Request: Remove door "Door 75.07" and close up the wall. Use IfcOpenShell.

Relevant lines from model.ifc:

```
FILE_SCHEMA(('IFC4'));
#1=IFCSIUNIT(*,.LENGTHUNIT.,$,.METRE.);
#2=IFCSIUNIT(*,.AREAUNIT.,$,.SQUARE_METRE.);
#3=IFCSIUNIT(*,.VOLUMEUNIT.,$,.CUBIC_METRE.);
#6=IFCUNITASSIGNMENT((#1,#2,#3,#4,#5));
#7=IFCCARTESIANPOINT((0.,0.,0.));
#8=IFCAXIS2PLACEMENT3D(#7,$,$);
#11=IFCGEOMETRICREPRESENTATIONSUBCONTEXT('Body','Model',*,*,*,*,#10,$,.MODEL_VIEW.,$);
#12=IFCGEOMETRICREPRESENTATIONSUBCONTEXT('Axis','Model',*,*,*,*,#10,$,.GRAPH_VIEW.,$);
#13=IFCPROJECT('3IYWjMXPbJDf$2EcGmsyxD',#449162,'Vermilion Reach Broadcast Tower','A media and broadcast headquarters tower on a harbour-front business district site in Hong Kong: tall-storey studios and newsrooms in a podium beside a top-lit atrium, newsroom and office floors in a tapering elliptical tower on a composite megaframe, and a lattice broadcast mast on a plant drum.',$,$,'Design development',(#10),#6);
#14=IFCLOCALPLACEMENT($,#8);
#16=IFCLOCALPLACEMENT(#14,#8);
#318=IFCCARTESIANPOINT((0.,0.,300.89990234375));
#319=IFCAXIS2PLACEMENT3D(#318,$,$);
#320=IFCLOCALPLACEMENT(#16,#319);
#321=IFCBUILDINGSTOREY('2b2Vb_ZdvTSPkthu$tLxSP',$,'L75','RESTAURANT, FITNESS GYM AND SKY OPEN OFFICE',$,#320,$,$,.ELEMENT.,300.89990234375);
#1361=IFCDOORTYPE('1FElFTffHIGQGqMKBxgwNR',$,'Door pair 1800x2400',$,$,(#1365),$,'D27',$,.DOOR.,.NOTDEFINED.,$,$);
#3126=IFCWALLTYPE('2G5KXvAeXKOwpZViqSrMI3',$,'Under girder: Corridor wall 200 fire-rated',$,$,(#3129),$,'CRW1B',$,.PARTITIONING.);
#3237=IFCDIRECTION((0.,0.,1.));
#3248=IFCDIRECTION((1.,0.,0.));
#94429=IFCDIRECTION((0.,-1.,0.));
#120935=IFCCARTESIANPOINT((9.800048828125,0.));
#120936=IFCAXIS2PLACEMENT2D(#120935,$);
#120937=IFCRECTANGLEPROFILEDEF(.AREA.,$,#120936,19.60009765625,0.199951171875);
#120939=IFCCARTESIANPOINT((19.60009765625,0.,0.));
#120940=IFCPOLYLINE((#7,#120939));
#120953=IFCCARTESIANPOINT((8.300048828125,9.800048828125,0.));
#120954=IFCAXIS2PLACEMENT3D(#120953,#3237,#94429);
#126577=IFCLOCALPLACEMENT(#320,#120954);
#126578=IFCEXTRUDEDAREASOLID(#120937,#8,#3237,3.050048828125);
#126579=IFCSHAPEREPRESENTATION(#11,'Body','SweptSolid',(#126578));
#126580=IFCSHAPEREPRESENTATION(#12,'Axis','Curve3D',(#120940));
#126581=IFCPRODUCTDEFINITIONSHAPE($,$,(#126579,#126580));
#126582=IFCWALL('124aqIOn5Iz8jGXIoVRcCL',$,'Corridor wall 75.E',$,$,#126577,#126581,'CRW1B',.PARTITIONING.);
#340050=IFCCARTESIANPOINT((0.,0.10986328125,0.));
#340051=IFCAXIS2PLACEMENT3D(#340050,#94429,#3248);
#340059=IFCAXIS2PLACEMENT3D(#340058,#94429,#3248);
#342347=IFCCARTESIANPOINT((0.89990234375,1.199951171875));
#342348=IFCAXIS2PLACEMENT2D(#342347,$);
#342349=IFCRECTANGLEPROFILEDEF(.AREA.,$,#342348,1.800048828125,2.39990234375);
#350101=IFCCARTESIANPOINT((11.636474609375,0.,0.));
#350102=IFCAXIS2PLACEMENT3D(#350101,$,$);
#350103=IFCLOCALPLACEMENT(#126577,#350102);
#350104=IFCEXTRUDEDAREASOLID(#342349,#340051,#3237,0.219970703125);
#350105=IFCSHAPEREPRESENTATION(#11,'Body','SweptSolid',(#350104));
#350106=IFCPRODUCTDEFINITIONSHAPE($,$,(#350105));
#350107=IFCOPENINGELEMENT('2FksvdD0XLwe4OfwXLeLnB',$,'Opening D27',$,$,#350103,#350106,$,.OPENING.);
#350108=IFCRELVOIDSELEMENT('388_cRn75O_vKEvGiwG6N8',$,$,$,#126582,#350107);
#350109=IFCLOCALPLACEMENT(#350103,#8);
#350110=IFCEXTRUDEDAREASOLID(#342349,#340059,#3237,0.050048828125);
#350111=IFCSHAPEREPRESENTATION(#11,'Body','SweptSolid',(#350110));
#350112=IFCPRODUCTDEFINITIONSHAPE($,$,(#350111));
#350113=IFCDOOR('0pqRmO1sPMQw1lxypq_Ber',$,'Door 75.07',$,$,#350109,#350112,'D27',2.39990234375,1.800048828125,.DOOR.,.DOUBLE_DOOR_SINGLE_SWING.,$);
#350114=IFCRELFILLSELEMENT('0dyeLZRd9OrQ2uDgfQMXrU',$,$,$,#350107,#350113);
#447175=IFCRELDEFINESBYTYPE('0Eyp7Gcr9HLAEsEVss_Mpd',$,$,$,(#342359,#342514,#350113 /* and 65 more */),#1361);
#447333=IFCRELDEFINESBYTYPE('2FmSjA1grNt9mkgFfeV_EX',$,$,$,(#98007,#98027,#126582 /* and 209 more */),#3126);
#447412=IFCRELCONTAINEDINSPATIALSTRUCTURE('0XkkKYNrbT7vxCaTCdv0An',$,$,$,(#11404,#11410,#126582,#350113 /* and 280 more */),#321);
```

```python
import ifcopenshell
import ifcopenshell.api.feature
import ifcopenshell.api.root
import ifcopenshell.geom
import ifcopenshell.util.shape

model = ifcopenshell.open("model.ifc")
settings = ifcopenshell.geom.settings()


def volume(element):
    """Net volume in cubic metres, openings subtracted."""
    shape = ifcopenshell.geom.create_shape(settings, element)
    return ifcopenshell.util.shape.get_volume(shape.geometry)


door = model.by_id(350113)
opening = door.FillsVoids[0].RelatingOpeningElement
wall = opening.VoidsElements[0].RelatingBuildingElement
before = volume(wall)

ifcopenshell.api.root.remove_product(model, product=door)
ifcopenshell.api.feature.remove_feature(model, feature=opening)

after = volume(wall)

print(f"wall volume {before:.3f} -> {after:.3f} m3")

model.write("model_updated.ifc")
```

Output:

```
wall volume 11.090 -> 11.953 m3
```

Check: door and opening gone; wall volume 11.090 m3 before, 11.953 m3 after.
